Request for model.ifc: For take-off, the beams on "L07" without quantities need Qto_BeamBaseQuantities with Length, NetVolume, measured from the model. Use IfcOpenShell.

First a look at what the model holds.

```python
import ifcopenshell
import ifcopenshell.util.element
import ifcopenshell.util.unit

model = ifcopenshell.open("model.ifc")
print(model.schema)
for unit_type in ("LENGTHUNIT", "AREAUNIT", "VOLUMEUNIT"):
    print(unit_type, ifcopenshell.util.unit.calculate_unit_scale(model, unit_type))
storey = next(s for s in model.by_type("IfcBuildingStorey") if s.Name == "L07")
beams = [e for e in ifcopenshell.util.element.get_decomposition(storey) if e.is_a("IfcBeam")]
for e in sorted(beams, key=lambda e: e.id()):
    print(e.id(), e.is_a(), e.Name, list(ifcopenshell.util.element.get_psets(e, qtos_only=True)), sep=" | ")
```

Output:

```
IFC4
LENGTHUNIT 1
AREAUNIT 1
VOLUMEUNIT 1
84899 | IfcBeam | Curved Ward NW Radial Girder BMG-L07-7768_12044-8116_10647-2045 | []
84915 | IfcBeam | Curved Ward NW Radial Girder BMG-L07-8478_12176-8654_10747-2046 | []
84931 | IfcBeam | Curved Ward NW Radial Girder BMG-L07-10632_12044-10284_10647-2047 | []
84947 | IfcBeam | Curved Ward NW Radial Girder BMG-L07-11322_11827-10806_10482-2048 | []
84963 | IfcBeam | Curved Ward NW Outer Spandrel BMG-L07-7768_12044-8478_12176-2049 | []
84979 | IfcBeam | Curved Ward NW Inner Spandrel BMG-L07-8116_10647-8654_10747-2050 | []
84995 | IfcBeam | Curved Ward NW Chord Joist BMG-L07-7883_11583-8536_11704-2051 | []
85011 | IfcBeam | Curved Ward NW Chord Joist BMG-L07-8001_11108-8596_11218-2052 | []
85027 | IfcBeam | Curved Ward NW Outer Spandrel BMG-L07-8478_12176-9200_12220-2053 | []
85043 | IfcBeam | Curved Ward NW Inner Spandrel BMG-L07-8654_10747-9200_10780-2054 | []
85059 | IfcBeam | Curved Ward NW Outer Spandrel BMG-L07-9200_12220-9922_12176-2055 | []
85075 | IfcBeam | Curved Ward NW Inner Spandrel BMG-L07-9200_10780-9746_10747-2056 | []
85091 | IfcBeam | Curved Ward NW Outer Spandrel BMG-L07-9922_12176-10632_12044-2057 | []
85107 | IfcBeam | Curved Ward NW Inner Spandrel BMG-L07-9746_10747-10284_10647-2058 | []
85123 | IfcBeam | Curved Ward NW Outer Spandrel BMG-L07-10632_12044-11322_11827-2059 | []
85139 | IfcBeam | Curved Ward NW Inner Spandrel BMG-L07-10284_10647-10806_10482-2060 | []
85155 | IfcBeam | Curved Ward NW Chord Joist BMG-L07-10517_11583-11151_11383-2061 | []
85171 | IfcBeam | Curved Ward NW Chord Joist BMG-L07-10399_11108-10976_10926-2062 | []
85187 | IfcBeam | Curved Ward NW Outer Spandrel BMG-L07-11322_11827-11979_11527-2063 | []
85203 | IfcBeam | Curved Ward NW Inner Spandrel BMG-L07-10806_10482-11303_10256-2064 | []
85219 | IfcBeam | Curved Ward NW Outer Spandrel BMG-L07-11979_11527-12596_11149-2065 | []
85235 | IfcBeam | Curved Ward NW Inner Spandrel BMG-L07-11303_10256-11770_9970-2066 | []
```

```python
import ifcopenshell
import ifcopenshell.api.pset
import ifcopenshell.geom
import ifcopenshell.util.element
import ifcopenshell.util.shape
import ifcopenshell.util.unit

model = ifcopenshell.open("model.ifc")
unit_scale = ifcopenshell.util.unit.calculate_unit_scale(model)
volume_scale = ifcopenshell.util.unit.calculate_unit_scale(model, "VOLUMEUNIT")
settings = ifcopenshell.geom.settings()

storey = next(s for s in model.by_type("IfcBuildingStorey") if s.Name == "L07")
beams = [e for e in ifcopenshell.util.element.get_decomposition(storey) if e.is_a("IfcBeam")]

for e in sorted(beams, key=lambda e: e.id()):
    if ifcopenshell.util.element.get_psets(e, qtos_only=True, should_inherit=False):
        continue
    # Geometry comes back in metres, in the element's own axes.
    shape = ifcopenshell.geom.create_shape(settings, e)
    values = {
        "Length": ifcopenshell.util.shape.get_max_xyz(shape.geometry) / unit_scale,
        "NetVolume": ifcopenshell.util.shape.get_volume(shape.geometry) / volume_scale,
    }
    qto = ifcopenshell.api.pset.add_qto(model, product=e, name="Qto_BeamBaseQuantities")
    ifcopenshell.api.pset.edit_qto(model, qto=qto, properties=values)
    print(e.id(), {k: round(v, 3) for k, v in values.items()})

model.write("model_v2.ifc")
```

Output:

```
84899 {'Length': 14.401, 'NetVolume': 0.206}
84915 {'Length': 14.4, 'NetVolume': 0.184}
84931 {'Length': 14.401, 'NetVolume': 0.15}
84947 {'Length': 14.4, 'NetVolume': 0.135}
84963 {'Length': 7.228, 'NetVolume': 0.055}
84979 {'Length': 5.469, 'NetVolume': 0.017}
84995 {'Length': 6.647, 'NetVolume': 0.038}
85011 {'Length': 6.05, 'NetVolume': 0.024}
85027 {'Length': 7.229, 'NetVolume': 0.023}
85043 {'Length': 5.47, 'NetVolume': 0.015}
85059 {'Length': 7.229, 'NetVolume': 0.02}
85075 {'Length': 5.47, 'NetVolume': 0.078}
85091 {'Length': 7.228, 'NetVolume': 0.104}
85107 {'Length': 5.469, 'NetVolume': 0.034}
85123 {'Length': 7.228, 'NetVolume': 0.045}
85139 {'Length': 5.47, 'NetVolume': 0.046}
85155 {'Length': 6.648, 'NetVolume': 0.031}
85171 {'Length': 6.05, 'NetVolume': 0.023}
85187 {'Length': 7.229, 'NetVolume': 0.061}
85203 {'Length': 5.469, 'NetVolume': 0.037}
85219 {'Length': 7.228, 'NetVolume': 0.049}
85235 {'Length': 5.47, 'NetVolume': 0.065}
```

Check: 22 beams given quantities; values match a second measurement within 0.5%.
